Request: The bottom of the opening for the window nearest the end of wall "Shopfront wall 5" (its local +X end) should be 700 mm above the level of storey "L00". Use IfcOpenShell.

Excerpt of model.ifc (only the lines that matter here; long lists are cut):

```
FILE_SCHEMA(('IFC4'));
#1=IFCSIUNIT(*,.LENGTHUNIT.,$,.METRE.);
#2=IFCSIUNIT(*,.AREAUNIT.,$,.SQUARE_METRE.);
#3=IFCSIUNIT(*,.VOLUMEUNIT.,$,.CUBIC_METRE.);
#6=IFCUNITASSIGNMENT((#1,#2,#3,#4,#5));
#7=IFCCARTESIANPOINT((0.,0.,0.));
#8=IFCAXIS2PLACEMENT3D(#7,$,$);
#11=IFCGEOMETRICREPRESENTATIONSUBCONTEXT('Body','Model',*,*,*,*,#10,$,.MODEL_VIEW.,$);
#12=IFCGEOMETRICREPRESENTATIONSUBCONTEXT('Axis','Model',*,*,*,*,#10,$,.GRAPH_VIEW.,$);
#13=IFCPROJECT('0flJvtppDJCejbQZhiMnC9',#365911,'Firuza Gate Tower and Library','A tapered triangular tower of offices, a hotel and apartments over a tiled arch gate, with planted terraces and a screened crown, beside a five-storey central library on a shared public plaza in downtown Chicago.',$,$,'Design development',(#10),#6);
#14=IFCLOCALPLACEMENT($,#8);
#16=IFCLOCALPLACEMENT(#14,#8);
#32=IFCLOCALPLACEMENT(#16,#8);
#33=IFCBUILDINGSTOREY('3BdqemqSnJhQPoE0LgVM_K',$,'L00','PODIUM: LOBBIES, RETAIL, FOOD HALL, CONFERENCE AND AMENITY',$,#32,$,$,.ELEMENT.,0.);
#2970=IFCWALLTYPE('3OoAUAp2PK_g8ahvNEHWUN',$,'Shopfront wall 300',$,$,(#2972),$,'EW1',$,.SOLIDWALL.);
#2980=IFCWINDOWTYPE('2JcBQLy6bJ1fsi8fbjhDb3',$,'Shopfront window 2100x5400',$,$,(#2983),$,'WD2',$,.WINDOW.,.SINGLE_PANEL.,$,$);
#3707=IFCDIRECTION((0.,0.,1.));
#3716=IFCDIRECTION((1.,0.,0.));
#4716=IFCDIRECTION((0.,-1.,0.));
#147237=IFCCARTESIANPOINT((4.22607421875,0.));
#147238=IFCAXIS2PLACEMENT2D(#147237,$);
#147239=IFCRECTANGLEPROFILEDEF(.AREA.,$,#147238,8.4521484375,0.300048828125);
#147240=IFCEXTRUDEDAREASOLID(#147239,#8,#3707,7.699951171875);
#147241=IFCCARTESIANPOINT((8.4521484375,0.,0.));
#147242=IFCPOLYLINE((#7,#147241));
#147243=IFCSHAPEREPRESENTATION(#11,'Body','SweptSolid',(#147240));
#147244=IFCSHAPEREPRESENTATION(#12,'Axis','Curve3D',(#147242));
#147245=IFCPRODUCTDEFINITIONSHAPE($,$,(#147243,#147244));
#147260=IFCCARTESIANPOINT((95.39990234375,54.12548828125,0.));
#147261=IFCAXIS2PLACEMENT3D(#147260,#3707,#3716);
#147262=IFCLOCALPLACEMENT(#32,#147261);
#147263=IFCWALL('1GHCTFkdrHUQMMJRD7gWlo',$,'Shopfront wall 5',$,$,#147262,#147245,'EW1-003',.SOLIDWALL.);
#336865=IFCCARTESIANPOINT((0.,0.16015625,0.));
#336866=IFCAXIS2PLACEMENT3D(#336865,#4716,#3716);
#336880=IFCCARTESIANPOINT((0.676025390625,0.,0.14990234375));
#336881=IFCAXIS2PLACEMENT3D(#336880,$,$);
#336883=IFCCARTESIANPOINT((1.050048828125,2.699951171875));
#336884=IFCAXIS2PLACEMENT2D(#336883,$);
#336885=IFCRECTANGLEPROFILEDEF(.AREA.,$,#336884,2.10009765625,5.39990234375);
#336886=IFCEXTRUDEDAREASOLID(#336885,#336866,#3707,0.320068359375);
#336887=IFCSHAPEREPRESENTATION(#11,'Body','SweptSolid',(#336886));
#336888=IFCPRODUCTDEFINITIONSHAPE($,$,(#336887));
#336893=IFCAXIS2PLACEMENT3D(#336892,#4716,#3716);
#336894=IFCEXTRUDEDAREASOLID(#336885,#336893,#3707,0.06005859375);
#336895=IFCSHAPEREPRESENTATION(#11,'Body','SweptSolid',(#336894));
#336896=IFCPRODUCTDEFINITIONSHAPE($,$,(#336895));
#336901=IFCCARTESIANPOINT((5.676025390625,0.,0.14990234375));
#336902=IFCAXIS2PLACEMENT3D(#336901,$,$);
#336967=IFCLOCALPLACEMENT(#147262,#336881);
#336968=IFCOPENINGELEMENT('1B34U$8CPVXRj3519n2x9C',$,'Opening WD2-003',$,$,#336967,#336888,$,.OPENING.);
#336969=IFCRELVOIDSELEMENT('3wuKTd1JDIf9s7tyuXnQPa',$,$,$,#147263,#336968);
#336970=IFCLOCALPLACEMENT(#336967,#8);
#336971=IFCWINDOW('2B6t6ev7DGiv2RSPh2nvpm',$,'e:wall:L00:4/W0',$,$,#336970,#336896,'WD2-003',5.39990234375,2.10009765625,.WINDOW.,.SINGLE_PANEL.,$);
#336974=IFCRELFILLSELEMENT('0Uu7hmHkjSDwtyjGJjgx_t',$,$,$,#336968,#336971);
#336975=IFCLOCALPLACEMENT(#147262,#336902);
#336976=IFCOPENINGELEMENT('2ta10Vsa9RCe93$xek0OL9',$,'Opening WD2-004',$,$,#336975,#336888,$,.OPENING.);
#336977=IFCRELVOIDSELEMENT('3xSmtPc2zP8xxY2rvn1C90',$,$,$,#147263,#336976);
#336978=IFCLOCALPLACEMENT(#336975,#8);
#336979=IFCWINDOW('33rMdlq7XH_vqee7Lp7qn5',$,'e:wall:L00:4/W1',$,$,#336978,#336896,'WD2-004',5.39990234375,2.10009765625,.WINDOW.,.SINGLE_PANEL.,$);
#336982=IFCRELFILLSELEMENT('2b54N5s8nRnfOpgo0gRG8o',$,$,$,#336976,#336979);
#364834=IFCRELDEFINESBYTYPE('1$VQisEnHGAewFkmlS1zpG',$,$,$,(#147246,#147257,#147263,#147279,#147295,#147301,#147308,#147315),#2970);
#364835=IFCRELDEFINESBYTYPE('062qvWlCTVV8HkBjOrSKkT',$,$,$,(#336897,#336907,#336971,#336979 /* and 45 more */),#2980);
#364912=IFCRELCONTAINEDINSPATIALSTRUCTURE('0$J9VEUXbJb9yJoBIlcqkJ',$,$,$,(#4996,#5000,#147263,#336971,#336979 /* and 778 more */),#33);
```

```python
import numpy as np
import ifcopenshell
import ifcopenshell.api.geometry
import ifcopenshell.geom
import ifcopenshell.util.element
import ifcopenshell.util.placement
import ifcopenshell.util.shape
import ifcopenshell.util.unit

model = ifcopenshell.open("model.ifc")
unit_scale = ifcopenshell.util.unit.calculate_unit_scale(model)

window = model.by_id(336979)
opening = window.FillsVoids[0].RelatingOpeningElement
storey = ifcopenshell.util.element.get_container(window, ifc_class="IfcBuildingStorey")
level = ifcopenshell.util.placement.get_local_placement(storey.ObjectPlacement)[2, 3]

# The opening's origin need not be at the sill, so measure its lowest point.
shape = ifcopenshell.geom.create_shape(ifcopenshell.geom.settings(), opening)
bottom = ifcopenshell.util.shape.get_shape_bottom_elevation(shape, shape.geometry) / unit_scale
dz = level + 0.7 / unit_scale - bottom

shift = np.array([0.0, 0.0, dz])
# The window is placed relative to its opening, so it follows when the opening moves.
matrix = ifcopenshell.util.placement.get_local_placement(opening.ObjectPlacement)
matrix[:3, 3] += shift
ifcopenshell.api.geometry.edit_object_placement(
    model, product=opening, matrix=matrix, is_si=False, should_transform_children=True
)

print(f"moved by {dz * unit_scale:+.3f} m")

model.write("model-out.ifc")
```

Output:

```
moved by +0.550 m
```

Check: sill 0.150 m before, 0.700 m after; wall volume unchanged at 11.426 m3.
